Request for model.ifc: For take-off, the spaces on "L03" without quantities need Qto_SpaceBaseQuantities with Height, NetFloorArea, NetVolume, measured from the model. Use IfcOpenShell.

First a look at what the model holds.

```python
import ifcopenshell
import ifcopenshell.util.element
import ifcopenshell.util.unit

model = ifcopenshell.open("model.ifc")
print(model.schema)
for unit_type in ("LENGTHUNIT", "AREAUNIT", "VOLUMEUNIT"):
    print(unit_type, ifcopenshell.util.unit.calculate_unit_scale(model, unit_type))
storey = next(s for s in model.by_type("IfcBuildingStorey") if s.Name == "L03")
spaces = [e for e in ifcopenshell.util.element.get_decomposition(storey) if e.is_a("IfcSpace")]
for e in sorted(spaces, key=lambda e: e.id()):
    print(e.id(), e.is_a(), e.Name, list(ifcopenshell.util.element.get_psets(e, qtos_only=True)), sep=" | ")
```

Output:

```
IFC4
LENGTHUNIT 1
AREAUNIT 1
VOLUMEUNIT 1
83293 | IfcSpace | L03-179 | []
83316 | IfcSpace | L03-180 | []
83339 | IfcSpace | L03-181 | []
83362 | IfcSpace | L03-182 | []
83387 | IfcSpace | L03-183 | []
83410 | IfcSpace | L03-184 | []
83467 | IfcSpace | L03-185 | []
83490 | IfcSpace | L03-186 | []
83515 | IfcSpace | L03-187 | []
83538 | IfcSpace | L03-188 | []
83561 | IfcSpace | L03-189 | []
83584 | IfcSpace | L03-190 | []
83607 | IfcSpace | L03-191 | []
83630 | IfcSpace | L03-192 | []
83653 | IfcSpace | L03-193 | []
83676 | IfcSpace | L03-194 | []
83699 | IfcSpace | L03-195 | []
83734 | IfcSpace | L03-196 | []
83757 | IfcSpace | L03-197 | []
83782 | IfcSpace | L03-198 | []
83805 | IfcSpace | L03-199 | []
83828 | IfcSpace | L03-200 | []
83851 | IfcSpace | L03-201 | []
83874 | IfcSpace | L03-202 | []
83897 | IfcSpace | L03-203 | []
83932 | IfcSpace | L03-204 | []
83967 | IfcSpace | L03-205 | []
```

```python
import ifcopenshell
import ifcopenshell.api.pset
import ifcopenshell.geom
import ifcopenshell.util.element
import ifcopenshell.util.shape
import ifcopenshell.util.unit

model = ifcopenshell.open("model.ifc")
unit_scale = ifcopenshell.util.unit.calculate_unit_scale(model)
area_scale = ifcopenshell.util.unit.calculate_unit_scale(model, "AREAUNIT")
volume_scale = ifcopenshell.util.unit.calculate_unit_scale(model, "VOLUMEUNIT")
settings = ifcopenshell.geom.settings()

storey = next(s for s in model.by_type("IfcBuildingStorey") if s.Name == "L03")
spaces = [e for e in ifcopenshell.util.element.get_decomposition(storey) if e.is_a("IfcSpace")]

for e in sorted(spaces, key=lambda e: e.id()):
    if ifcopenshell.util.element.get_psets(e, qtos_only=True, should_inherit=False):
        continue
    # Geometry comes back in metres, in the element's own axes.
    shape = ifcopenshell.geom.create_shape(settings, e)
    values = {
        "Height": ifcopenshell.util.shape.get_z(shape.geometry) / unit_scale,
        "NetFloorArea": ifcopenshell.util.shape.get_footprint_area(shape.geometry) / area_scale,
        "NetVolume": ifcopenshell.util.shape.get_volume(shape.geometry) / volume_scale,
    }
    qto = ifcopenshell.api.pset.add_qto(model, product=e, name="Qto_SpaceBaseQuantities")
    ifcopenshell.api.pset.edit_qto(model, qto=qto, properties=values)
    print(e.id(), {k: round(v, 3) for k, v in values.items()})

model.write("model_rev.ifc")
```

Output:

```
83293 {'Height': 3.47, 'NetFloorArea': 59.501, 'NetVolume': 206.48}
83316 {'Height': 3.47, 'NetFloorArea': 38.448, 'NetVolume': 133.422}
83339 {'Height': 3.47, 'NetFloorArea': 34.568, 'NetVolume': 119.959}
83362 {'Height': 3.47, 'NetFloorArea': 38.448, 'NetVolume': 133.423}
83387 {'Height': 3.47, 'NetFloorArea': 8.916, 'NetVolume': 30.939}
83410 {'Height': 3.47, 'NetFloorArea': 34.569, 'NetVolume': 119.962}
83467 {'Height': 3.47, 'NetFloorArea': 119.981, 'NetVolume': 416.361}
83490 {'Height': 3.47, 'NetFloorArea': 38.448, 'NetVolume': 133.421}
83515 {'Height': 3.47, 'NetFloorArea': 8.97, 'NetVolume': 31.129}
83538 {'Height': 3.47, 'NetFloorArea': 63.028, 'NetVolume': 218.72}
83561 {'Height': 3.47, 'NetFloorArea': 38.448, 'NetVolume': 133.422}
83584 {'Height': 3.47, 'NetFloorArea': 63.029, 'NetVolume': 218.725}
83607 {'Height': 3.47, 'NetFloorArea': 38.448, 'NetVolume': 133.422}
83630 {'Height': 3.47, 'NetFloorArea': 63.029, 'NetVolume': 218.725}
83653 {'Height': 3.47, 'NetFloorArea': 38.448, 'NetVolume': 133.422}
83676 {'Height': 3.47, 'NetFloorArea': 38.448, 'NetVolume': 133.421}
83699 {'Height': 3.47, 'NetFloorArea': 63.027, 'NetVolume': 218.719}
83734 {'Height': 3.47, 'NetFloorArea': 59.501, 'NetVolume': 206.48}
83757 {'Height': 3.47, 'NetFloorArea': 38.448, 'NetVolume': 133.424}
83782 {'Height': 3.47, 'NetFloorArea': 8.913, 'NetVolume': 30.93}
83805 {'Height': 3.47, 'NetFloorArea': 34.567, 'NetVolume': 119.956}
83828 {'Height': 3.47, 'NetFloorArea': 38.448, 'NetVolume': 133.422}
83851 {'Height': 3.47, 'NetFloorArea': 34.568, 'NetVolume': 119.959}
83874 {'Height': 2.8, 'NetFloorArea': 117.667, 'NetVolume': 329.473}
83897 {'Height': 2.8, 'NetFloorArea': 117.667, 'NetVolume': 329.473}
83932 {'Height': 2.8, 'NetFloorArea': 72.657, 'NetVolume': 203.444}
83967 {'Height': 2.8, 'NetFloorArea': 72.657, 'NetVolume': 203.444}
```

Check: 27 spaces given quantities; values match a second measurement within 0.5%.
